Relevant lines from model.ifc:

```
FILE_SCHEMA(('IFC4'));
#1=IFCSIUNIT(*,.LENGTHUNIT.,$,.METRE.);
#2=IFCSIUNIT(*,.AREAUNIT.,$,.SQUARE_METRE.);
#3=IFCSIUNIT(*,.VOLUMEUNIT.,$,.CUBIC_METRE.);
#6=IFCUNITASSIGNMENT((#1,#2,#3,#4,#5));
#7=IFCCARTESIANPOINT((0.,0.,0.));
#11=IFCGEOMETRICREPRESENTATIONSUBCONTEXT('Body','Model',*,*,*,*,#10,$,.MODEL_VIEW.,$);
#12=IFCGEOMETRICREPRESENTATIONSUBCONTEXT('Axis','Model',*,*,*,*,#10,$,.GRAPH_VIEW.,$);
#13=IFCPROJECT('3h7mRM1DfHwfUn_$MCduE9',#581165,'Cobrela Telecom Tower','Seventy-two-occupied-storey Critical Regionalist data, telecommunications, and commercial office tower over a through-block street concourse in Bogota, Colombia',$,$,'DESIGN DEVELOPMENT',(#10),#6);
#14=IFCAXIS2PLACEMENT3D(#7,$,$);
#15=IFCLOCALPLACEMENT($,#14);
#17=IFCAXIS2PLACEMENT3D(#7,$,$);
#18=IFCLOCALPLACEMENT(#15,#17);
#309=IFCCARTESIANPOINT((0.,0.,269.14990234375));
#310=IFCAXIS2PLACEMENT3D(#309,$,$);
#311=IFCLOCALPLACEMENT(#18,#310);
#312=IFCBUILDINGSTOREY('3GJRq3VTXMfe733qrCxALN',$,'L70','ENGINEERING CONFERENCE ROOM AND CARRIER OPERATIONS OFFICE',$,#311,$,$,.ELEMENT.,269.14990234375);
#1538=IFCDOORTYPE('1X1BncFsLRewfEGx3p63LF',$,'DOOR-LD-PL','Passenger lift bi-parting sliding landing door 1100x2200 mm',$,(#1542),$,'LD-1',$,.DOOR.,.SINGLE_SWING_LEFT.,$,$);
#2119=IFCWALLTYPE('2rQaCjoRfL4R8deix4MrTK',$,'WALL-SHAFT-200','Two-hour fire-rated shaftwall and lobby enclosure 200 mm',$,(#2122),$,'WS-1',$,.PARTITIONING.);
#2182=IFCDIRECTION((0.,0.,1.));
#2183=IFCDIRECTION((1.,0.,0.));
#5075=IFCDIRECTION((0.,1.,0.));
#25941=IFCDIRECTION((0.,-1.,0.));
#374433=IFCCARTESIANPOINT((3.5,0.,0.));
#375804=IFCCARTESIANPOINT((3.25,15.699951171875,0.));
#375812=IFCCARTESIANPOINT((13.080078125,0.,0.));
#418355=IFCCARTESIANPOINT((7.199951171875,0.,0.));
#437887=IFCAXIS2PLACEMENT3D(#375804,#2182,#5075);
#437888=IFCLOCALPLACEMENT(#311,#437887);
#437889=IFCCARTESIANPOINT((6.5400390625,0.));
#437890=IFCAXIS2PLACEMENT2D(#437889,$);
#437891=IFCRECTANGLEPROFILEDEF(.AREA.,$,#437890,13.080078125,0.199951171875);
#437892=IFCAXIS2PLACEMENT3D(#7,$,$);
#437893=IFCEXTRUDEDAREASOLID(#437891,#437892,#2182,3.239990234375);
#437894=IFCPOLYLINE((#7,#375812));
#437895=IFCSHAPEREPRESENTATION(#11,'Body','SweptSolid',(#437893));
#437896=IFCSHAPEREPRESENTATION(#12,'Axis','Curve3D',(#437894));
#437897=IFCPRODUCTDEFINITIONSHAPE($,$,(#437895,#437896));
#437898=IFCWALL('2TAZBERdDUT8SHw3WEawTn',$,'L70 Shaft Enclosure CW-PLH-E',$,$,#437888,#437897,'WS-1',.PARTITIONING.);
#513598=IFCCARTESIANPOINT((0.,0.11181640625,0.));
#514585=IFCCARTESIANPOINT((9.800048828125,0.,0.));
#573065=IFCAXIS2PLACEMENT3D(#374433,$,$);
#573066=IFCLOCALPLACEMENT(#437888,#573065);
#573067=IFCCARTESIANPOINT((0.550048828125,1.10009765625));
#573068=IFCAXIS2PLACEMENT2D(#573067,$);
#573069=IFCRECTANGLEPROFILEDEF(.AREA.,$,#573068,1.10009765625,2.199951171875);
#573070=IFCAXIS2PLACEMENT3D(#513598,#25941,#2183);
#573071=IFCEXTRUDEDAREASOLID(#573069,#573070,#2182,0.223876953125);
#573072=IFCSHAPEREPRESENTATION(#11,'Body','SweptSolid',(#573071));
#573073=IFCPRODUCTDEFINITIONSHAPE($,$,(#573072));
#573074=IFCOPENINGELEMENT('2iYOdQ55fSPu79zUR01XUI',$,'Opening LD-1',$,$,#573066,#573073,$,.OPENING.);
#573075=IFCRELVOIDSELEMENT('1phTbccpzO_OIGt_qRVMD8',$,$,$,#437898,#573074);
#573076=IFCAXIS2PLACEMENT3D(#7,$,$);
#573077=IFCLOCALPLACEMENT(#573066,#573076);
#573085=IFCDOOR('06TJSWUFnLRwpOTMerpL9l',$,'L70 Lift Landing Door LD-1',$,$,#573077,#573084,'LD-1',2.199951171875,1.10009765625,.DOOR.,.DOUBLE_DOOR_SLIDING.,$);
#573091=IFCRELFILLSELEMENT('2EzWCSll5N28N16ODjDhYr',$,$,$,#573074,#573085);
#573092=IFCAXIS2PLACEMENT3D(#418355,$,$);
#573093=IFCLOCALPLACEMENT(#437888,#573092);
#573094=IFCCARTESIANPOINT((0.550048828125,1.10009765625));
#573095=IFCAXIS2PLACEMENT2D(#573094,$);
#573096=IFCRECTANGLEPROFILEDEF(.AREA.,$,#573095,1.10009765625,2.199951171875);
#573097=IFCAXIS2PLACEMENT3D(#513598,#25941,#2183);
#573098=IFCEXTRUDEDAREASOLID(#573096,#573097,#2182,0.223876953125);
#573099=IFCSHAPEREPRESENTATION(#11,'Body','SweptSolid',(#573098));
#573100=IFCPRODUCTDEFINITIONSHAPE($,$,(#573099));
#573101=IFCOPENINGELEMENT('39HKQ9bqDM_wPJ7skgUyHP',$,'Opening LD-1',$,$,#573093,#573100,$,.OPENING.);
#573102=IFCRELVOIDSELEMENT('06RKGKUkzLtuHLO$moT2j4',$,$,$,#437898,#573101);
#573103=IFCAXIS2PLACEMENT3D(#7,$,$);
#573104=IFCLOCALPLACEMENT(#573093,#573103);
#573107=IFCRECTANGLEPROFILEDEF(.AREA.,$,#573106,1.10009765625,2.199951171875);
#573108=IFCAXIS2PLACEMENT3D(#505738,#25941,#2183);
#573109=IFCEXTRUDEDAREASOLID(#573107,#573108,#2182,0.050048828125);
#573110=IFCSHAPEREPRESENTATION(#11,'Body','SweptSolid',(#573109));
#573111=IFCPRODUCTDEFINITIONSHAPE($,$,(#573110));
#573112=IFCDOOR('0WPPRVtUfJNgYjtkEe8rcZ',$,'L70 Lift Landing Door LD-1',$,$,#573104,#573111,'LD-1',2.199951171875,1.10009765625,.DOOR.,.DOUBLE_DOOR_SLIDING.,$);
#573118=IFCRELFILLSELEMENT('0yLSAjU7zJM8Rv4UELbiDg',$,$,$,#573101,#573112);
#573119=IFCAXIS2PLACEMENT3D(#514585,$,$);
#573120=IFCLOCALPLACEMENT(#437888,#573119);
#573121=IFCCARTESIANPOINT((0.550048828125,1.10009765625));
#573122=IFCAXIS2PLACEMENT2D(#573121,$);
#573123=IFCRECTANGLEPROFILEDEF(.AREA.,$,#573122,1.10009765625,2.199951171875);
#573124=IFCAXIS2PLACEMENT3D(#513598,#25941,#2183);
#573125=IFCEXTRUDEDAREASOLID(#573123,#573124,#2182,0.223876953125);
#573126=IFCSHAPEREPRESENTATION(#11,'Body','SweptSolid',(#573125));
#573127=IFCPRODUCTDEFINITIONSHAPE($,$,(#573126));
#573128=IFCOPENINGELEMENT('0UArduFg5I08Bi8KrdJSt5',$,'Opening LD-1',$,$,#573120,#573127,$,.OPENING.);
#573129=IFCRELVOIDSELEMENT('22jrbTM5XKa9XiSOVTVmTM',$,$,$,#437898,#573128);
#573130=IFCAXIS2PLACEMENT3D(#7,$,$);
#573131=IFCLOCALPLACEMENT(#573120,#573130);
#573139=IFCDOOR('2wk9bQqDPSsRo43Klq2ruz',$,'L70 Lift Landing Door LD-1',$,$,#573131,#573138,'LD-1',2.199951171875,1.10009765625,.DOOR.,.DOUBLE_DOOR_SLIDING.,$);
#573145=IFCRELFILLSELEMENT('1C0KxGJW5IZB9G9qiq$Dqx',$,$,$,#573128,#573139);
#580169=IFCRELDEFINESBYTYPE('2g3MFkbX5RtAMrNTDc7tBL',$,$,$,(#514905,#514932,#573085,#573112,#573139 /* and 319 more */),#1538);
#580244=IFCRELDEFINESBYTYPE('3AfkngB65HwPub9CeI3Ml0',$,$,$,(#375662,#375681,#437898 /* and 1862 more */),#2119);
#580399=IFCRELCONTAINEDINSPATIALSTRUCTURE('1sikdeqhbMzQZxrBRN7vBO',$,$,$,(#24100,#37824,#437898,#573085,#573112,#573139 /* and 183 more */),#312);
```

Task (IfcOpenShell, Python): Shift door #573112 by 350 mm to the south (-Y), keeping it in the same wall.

```python
import ifcopenshell
import ifcopenshell.api.geometry
import ifcopenshell.util.placement

model = ifcopenshell.open("model.ifc")

door = model.by_id(573112)
opening = door.FillsVoids[0].RelatingOpeningElement
wall = opening.VoidsElements[0].RelatingBuildingElement

wall_matrix = ifcopenshell.util.placement.get_local_placement(wall.ObjectPlacement)
shift = wall_matrix[:3, 0] * -0.35
before = ifcopenshell.util.placement.get_local_placement(door.ObjectPlacement)[:3, 3].copy()

# The door is placed relative to its opening, so it follows when the opening moves.
matrix = ifcopenshell.util.placement.get_local_placement(opening.ObjectPlacement)
matrix[:3, 3] += shift
ifcopenshell.api.geometry.edit_object_placement(
    model, product=opening, matrix=matrix, is_si=False, should_transform_children=True
)

after = ifcopenshell.util.placement.get_local_placement(door.ObjectPlacement)[:3, 3]
print("door moved by", (after - before).round(3) + 0.0)

model.write("model_rev.ifc")
```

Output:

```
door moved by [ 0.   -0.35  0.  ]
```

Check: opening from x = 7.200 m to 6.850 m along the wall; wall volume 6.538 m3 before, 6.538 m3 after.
